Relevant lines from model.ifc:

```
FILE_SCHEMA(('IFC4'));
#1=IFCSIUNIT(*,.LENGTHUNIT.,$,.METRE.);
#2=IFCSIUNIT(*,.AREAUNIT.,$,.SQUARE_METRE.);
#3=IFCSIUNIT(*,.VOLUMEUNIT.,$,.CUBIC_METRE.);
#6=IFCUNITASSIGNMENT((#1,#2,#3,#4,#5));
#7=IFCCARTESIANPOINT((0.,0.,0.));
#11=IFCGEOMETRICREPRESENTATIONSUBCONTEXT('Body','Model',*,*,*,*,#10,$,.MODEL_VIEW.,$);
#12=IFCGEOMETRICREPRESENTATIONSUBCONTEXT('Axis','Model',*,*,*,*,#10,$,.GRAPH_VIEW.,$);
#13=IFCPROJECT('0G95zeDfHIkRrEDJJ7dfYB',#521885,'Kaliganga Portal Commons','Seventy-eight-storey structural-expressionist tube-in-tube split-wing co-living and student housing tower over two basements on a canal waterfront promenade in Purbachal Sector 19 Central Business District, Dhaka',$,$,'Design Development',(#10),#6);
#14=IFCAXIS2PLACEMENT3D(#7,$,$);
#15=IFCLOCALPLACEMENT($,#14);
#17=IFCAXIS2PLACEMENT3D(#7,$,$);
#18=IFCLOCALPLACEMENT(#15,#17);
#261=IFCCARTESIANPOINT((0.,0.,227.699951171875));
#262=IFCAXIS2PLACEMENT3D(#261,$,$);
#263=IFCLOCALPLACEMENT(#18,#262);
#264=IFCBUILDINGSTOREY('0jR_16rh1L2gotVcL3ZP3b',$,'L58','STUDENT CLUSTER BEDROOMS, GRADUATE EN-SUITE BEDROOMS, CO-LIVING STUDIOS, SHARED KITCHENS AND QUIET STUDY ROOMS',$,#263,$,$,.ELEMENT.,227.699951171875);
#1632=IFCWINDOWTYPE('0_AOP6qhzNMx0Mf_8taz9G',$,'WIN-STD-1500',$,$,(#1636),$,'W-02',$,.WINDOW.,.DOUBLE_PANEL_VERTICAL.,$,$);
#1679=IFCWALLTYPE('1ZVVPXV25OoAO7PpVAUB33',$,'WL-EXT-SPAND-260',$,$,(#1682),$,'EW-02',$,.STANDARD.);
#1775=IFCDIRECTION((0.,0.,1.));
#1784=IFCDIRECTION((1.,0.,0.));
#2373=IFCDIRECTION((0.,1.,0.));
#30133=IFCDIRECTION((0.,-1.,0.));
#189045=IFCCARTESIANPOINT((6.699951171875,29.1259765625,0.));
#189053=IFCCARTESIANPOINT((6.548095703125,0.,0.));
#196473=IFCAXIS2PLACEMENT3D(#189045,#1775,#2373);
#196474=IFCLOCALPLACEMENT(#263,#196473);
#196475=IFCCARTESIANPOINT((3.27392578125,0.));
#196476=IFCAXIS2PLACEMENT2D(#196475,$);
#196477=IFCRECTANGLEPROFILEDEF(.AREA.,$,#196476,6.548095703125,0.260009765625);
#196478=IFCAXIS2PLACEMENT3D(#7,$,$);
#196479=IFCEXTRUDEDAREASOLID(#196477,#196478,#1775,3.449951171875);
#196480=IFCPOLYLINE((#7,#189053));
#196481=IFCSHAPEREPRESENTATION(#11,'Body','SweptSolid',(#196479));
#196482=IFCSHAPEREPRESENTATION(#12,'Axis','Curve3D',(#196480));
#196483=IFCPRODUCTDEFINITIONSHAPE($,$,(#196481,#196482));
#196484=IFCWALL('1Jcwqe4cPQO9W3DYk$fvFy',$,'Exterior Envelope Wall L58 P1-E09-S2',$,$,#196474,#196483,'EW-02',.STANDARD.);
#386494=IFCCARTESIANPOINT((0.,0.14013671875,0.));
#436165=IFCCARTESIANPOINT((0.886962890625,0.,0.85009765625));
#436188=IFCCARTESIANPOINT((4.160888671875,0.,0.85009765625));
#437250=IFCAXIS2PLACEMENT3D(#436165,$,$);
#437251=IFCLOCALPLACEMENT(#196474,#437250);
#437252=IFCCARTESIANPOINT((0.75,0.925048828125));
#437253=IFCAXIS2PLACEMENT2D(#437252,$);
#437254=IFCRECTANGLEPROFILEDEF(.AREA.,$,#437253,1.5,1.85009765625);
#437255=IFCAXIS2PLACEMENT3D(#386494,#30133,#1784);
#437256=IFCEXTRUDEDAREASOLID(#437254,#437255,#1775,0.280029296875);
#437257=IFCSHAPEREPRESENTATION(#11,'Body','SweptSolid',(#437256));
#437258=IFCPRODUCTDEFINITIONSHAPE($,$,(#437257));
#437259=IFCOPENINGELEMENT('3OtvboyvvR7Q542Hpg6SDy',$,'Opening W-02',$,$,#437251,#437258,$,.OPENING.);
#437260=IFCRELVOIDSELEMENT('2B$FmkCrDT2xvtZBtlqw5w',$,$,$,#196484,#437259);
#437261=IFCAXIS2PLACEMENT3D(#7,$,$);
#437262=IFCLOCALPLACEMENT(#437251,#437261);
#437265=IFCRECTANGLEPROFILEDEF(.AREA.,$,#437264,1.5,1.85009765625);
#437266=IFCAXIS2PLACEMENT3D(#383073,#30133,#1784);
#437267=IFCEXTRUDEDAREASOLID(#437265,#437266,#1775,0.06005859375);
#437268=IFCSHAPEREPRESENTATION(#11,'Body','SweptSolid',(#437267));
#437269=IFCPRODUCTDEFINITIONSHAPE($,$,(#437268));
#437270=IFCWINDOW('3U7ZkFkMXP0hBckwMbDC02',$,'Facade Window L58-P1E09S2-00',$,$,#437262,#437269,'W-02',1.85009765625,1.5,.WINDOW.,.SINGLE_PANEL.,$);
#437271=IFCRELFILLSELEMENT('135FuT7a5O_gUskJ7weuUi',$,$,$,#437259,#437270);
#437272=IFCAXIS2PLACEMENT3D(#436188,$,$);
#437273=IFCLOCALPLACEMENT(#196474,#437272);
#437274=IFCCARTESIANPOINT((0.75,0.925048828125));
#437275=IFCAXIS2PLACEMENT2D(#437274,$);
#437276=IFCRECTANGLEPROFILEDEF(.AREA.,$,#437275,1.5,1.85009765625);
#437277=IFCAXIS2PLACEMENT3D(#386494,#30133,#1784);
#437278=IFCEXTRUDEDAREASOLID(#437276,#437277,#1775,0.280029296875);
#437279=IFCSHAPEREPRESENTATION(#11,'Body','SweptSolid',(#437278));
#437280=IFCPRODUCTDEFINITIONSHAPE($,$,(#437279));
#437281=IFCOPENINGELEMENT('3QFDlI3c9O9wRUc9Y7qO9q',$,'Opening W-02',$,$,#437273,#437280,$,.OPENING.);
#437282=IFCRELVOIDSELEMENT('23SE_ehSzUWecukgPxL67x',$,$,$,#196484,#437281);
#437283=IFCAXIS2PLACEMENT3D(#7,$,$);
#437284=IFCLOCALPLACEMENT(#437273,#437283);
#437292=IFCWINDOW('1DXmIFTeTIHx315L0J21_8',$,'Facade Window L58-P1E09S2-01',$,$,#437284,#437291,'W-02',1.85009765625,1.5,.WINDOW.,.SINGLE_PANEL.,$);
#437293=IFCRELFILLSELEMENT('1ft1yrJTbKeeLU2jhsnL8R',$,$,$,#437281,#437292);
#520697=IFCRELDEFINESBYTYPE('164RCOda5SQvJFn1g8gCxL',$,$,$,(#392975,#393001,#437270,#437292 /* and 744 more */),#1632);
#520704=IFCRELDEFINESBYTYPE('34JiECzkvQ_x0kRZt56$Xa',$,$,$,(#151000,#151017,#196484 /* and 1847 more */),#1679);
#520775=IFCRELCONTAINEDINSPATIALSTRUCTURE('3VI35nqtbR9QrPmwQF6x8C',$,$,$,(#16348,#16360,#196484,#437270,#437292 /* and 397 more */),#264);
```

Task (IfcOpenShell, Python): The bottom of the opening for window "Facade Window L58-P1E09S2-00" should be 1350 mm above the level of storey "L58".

```python
import numpy as np
import ifcopenshell
import ifcopenshell.api.geometry
import ifcopenshell.geom
import ifcopenshell.util.element
import ifcopenshell.util.placement
import ifcopenshell.util.shape
import ifcopenshell.util.unit

model = ifcopenshell.open("model.ifc")
unit_scale = ifcopenshell.util.unit.calculate_unit_scale(model)

window = model.by_guid("3U7ZkFkMXP0hBckwMbDC02")
opening = window.FillsVoids[0].RelatingOpeningElement
storey = ifcopenshell.util.element.get_container(window, ifc_class="IfcBuildingStorey")
level = ifcopenshell.util.placement.get_local_placement(storey.ObjectPlacement)[2, 3]

# The opening's origin need not be at the sill, so measure its lowest point.
shape = ifcopenshell.geom.create_shape(ifcopenshell.geom.settings(), opening)
bottom = ifcopenshell.util.shape.get_shape_bottom_elevation(shape, shape.geometry) / unit_scale
dz = level + 1.35 - bottom

shift = np.array([0.0, 0.0, dz])
# The window is placed relative to its opening, so it follows when the opening moves.
matrix = ifcopenshell.util.placement.get_local_placement(opening.ObjectPlacement)
matrix[:3, 3] += shift
ifcopenshell.api.geometry.edit_object_placement(
    model, product=opening, matrix=matrix, is_si=False, should_transform_children=True
)

print(f"moved by {dz * unit_scale:+.3f} m")

model.write("model_v2.ifc")
```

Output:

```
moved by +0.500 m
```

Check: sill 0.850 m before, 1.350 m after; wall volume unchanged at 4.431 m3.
